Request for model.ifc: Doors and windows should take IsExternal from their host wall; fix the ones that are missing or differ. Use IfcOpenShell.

First a look at what the model holds.

```python
import ifcopenshell
import ifcopenshell.util.element

model = ifcopenshell.open("model.ifc")
print(model.schema)
seen = {}
for e in model.by_type("IfcDoor") + model.by_type("IfcWindow"):
    if not e.FillsVoids:
        continue
    host = e.FillsVoids[0].RelatingOpeningElement.VoidsElements[0].RelatingBuildingElement
    own = ifcopenshell.util.element.get_pset(e, f"Pset_{e.is_a()[3:].removesuffix('StandardCase')}Common", "IsExternal")
    wall = ifcopenshell.util.element.get_pset(host, "Pset_WallCommon", "IsExternal")
    seen[e.is_a(), own, wall] = seen.get((e.is_a(), own, wall), 0) + 1
for (cls, own, wall), count in sorted(seen.items(), key=str):
    print(count, cls, "IsExternal:", own, "| host wall:", wall)
```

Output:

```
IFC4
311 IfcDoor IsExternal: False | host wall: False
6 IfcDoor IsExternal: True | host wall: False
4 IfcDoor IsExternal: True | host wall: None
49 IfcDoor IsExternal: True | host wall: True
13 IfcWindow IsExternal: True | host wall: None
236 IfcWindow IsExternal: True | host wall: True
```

```python
import ifcopenshell
import ifcopenshell.api.pset
import ifcopenshell.util.element

model = ifcopenshell.open("model.ifc")

count = 0
for ifc_class, pset_name in (("IfcDoor", "Pset_DoorCommon"), ("IfcWindow", "Pset_WindowCommon")):
    for e in model.by_type(ifc_class):
        if not e.FillsVoids:
            continue
        host = e.FillsVoids[0].RelatingOpeningElement.VoidsElements[0].RelatingBuildingElement
        external = ifcopenshell.util.element.get_pset(host, "Pset_WallCommon", "IsExternal")
        if external is None or ifcopenshell.util.element.get_pset(e, pset_name, "IsExternal") == external:
            continue
        pset = ifcopenshell.api.pset.add_pset(model, product=e, name=pset_name)
        ifcopenshell.api.pset.edit_pset(model, pset=pset, properties={"IsExternal": external})
        count += 1

print(count, "updated")

model.write("model-out.ifc")
```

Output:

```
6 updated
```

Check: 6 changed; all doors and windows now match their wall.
